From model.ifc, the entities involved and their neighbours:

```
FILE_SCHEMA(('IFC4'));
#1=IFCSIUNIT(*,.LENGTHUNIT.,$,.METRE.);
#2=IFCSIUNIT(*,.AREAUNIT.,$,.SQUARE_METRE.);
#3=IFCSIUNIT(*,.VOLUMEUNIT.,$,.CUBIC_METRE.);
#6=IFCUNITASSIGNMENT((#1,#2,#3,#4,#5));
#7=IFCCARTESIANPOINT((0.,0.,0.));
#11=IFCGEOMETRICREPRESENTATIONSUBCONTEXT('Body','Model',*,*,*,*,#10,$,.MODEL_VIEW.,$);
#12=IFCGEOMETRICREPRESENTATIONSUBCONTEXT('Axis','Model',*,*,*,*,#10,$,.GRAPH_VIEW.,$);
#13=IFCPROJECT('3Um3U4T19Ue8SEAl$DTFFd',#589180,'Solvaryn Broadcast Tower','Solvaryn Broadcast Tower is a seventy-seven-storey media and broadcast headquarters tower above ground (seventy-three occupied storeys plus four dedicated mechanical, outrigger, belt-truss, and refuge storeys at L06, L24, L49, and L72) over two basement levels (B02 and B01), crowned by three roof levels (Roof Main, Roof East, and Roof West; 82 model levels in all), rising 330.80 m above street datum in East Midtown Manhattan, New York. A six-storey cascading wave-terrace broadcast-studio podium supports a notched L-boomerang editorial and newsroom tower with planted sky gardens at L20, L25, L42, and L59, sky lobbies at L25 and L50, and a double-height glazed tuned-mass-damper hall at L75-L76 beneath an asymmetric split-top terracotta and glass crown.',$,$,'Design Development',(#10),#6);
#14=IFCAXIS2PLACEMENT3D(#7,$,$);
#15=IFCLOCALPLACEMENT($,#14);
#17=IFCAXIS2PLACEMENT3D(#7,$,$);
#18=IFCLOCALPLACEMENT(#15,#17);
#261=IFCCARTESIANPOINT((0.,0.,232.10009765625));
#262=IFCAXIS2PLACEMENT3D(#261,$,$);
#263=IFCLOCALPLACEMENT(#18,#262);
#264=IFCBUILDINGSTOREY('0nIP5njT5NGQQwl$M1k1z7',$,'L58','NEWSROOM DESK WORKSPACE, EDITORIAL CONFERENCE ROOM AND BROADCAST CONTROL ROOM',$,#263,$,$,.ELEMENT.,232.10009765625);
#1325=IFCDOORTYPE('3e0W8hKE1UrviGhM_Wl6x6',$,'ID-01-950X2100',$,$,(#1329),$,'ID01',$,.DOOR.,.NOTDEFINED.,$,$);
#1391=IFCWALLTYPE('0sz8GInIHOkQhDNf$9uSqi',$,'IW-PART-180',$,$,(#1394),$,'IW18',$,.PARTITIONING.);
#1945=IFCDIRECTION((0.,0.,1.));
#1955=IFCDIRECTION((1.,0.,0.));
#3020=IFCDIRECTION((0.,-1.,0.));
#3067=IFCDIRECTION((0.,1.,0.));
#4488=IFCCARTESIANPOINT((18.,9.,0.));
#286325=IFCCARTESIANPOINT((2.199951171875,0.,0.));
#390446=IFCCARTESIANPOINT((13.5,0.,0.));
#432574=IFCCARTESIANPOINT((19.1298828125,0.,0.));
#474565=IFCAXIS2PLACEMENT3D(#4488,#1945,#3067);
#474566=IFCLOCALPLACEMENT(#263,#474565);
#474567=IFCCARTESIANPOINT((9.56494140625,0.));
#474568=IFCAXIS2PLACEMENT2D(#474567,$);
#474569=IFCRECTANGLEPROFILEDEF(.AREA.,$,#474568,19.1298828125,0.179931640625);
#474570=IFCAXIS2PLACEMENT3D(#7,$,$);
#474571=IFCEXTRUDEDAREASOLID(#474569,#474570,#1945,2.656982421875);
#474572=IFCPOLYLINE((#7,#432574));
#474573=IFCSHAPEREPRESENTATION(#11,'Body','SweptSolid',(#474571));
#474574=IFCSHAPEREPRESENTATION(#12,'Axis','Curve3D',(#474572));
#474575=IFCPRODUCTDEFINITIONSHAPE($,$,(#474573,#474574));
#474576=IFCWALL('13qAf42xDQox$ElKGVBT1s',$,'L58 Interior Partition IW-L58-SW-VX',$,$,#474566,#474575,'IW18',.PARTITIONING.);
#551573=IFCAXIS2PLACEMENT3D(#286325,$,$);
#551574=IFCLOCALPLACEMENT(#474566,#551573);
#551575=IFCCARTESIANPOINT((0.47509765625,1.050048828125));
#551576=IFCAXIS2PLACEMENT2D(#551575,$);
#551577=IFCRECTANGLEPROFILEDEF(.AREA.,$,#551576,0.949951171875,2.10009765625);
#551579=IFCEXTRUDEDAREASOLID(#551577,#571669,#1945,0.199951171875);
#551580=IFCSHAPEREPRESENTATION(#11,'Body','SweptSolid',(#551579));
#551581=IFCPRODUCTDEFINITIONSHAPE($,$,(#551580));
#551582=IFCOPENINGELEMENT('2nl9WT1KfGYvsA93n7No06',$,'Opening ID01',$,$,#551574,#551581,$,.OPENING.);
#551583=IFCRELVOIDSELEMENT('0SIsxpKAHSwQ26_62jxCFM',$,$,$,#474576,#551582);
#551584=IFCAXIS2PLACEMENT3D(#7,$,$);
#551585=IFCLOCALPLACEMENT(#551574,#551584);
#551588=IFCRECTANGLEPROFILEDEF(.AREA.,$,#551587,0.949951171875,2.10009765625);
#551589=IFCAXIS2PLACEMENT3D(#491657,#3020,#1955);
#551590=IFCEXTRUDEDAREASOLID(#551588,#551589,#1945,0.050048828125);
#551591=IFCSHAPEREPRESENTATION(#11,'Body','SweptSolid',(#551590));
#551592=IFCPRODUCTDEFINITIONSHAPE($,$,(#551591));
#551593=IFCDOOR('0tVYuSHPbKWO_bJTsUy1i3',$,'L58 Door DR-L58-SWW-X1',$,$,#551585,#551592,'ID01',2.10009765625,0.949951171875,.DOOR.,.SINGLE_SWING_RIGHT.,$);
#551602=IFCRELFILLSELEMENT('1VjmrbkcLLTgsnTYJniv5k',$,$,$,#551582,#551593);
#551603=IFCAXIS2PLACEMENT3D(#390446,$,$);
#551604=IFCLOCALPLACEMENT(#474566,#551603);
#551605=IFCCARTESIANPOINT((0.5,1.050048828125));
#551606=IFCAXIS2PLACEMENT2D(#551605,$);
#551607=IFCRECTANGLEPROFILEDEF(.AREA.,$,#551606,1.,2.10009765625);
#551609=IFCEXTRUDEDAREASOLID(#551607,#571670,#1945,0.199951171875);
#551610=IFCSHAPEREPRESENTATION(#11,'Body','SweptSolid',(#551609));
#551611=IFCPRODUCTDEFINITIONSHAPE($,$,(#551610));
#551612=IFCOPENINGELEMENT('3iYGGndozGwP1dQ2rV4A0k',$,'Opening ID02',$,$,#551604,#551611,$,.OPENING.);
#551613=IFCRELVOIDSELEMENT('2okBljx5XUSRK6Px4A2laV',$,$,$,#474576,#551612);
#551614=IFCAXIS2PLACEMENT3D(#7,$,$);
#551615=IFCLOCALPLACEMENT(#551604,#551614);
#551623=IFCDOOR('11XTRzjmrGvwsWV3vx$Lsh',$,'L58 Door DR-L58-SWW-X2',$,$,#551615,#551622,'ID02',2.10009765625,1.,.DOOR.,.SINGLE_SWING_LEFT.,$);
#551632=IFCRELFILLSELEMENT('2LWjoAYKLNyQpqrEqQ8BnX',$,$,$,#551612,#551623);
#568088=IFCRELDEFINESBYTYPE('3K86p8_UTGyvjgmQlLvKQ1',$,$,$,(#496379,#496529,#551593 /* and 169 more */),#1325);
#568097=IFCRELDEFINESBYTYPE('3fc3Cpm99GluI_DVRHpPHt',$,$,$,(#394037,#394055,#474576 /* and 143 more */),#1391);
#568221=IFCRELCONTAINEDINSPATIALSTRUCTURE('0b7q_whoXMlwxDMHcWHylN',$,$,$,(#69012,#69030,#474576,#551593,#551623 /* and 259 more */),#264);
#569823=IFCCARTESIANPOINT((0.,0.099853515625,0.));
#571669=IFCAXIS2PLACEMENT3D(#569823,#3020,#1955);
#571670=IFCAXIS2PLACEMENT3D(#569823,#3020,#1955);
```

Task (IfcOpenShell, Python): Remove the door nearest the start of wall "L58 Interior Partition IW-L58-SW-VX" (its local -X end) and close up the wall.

```python
import ifcopenshell
import ifcopenshell.api.feature
import ifcopenshell.api.root
import ifcopenshell.geom
import ifcopenshell.util.shape

model = ifcopenshell.open("model.ifc")
settings = ifcopenshell.geom.settings()


def volume(element):
    """Net volume in cubic metres, openings subtracted."""
    shape = ifcopenshell.geom.create_shape(settings, element)
    return ifcopenshell.util.shape.get_volume(shape.geometry)


door = model.by_guid("0tVYuSHPbKWO_bJTsUy1i3")
opening = door.FillsVoids[0].RelatingOpeningElement
wall = opening.VoidsElements[0].RelatingBuildingElement
before = volume(wall)

ifcopenshell.api.root.remove_product(model, product=door)
ifcopenshell.api.feature.remove_feature(model, feature=opening)

after = volume(wall)

print(f"wall volume {before:.3f} -> {after:.3f} m3")

model.write("model-out.ifc")
```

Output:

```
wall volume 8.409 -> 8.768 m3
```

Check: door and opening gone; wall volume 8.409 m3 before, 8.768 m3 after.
